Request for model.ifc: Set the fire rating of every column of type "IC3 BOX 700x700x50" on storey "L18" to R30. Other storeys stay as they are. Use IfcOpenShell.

First a look at what the model holds.

```python
import ifcopenshell
import ifcopenshell.util.element

model = ifcopenshell.open("model.ifc")
print(model.schema)
storey = next(s for s in model.by_type("IfcBuildingStorey") if s.Name == "L18")
columns = [e for e in ifcopenshell.util.element.get_decomposition(storey) if e.is_a("IfcColumn")]
seen = {}
for e in columns:
    element_type = ifcopenshell.util.element.get_type(e)
    key = (element_type.Name if element_type != e and element_type else None, ifcopenshell.util.element.get_pset(e, "Pset_ColumnCommon", "FireRating"))
    seen[key] = seen.get(key, 0) + 1
for (name, value), count in sorted(seen.items(), key=str):
    print(count, "x", name, "|", value)
```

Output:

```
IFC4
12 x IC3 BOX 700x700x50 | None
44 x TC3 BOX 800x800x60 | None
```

```python
import ifcopenshell
import ifcopenshell.api.pset
import ifcopenshell.util.element

model = ifcopenshell.open("model.ifc")

storey = next(s for s in model.by_type("IfcBuildingStorey") if s.Name == "L18")
columns = [e for e in ifcopenshell.util.element.get_decomposition(storey) if e.is_a("IfcColumn")]

count = 0
for e in columns:
    element_type = ifcopenshell.util.element.get_type(e)
    if element_type in (None, e) or element_type.Name != "IC3 BOX 700x700x50":
        continue
    found = ifcopenshell.util.element.get_pset(e, "Pset_ColumnCommon", should_inherit=False)
    if found:
        pset = model.by_id(found["id"])
        if len(ifcopenshell.util.element.get_elements_by_pset(pset)) > 1:
            pset = ifcopenshell.api.pset.unshare_pset(model, products=[e], pset=pset)[0]
    else:
        pset = ifcopenshell.api.pset.add_pset(model, product=e, name="Pset_ColumnCommon")
    ifcopenshell.api.pset.edit_pset(model, pset=pset, properties={"FireRating": "R30"})
    count += 1

print(count, "columns updated")

model.write("model_edited.ifc")
```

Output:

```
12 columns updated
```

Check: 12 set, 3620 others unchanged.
